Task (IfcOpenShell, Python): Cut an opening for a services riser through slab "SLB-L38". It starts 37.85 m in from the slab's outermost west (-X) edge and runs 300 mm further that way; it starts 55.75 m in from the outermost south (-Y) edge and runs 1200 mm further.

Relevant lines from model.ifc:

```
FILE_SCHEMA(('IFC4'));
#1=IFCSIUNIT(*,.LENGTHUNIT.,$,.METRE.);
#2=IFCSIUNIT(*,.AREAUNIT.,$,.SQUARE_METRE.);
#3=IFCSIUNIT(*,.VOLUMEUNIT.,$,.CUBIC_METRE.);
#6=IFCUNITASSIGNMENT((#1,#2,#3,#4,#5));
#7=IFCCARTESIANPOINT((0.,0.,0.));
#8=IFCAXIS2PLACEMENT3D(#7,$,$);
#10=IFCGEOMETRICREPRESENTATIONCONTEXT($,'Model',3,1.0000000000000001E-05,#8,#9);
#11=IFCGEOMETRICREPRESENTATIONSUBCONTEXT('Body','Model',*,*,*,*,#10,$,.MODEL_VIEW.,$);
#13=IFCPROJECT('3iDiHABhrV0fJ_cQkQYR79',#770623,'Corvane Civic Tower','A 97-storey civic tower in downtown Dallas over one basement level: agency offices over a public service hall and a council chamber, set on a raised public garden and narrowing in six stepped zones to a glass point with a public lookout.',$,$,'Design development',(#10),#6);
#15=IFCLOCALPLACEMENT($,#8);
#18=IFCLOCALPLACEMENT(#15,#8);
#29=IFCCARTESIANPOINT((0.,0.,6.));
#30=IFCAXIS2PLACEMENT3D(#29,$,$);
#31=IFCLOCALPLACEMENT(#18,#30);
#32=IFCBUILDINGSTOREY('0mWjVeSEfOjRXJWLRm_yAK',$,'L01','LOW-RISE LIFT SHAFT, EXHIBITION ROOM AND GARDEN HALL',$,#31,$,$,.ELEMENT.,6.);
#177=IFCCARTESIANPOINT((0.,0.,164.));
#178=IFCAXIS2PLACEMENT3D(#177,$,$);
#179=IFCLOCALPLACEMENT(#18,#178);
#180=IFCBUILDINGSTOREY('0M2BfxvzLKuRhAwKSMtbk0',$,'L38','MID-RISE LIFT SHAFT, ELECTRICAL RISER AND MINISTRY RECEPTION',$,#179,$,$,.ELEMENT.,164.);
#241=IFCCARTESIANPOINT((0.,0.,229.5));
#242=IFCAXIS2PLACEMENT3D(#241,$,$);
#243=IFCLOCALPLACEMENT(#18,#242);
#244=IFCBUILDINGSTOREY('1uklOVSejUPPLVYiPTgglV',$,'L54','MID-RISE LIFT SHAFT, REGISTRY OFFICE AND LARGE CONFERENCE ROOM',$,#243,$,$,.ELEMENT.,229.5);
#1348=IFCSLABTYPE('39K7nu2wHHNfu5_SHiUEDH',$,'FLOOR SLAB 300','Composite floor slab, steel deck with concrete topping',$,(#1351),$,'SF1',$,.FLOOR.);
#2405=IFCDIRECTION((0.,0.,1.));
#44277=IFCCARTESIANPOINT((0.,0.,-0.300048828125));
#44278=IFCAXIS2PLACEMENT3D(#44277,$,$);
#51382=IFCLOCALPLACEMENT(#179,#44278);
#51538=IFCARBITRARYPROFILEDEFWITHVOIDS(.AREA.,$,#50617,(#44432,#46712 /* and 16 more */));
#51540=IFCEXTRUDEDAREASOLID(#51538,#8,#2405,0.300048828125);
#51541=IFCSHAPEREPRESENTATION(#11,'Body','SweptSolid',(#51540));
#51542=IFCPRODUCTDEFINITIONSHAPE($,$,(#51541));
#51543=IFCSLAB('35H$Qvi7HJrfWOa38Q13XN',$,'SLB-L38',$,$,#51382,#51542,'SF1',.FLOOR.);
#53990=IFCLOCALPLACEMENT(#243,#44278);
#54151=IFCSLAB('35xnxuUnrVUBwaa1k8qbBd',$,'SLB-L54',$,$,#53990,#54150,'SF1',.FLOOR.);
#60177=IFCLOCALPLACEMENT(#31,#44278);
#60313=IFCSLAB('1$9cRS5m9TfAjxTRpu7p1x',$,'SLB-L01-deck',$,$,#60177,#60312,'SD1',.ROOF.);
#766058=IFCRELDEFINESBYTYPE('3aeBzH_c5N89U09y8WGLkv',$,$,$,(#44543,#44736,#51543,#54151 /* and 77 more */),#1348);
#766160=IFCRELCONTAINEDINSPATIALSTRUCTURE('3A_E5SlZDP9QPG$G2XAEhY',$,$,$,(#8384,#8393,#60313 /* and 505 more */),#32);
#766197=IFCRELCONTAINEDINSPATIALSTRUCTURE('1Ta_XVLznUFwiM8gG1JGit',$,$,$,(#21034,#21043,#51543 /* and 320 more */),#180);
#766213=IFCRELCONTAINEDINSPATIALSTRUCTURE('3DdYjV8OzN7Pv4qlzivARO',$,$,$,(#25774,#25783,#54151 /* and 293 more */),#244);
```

```python
import numpy as np
import ifcopenshell
import ifcopenshell.api.feature
import ifcopenshell.api.geometry
import ifcopenshell.api.root
import ifcopenshell.geom
import ifcopenshell.util.placement
import ifcopenshell.util.representation
import ifcopenshell.util.shape
import ifcopenshell.util.unit

model = ifcopenshell.open("model.ifc")
unit_scale = ifcopenshell.util.unit.calculate_unit_scale(model)
settings = ifcopenshell.geom.settings()


def volume(element):
    """Net volume in cubic metres, openings subtracted."""
    shape = ifcopenshell.geom.create_shape(settings, element)
    return ifcopenshell.util.shape.get_volume(shape.geometry)


slab = model.by_guid("35H$Qvi7HJrfWOa38Q13XN")
before = volume(slab)

# Extent in the slab's own axes, in metres. The edges named are its -X and -Y sides.
slab_shape = ifcopenshell.geom.create_shape(settings, slab)
vertices = ifcopenshell.util.shape.get_vertices(slab_shape.geometry)
x_min, y_min, bottom = vertices.min(axis=0)
top = vertices[:, 2].max()

opening = ifcopenshell.api.root.create_entity(model, ifc_class="IfcOpeningElement", name="Services riser opening", predefined_type="OPENING")
context = ifcopenshell.util.representation.get_context(model, "Model", "Body", "MODEL_VIEW")
width, depth = 0.3, 1.2
outline = [(0.0, 0.0), (width, 0.0), (width, depth), (0.0, depth), (0.0, 0.0)]
# Overshoot both faces by 50 mm so the cut is clean.
shape = ifcopenshell.api.geometry.add_slab_representation(
    model, context=context, depth=top - bottom + 0.1, polyline=outline
)
ifcopenshell.api.geometry.assign_representation(model, product=opening, representation=shape)

matrix = ifcopenshell.util.placement.get_local_placement(slab.ObjectPlacement)
matrix[:, 3] = matrix @ np.append(np.array([x_min + 37.85, y_min + 55.75, bottom - 0.05]) / unit_scale, 1.0)
ifcopenshell.api.geometry.edit_object_placement(model, product=opening, matrix=matrix, is_si=False)
ifcopenshell.api.feature.add_feature(model, feature=opening, element=slab)

after = volume(slab)

print(f"slab volume {before:.3f} -> {after:.3f} m3")

model.write("model_updated.ifc")
```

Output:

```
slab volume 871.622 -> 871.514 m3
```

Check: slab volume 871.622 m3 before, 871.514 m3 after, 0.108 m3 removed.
